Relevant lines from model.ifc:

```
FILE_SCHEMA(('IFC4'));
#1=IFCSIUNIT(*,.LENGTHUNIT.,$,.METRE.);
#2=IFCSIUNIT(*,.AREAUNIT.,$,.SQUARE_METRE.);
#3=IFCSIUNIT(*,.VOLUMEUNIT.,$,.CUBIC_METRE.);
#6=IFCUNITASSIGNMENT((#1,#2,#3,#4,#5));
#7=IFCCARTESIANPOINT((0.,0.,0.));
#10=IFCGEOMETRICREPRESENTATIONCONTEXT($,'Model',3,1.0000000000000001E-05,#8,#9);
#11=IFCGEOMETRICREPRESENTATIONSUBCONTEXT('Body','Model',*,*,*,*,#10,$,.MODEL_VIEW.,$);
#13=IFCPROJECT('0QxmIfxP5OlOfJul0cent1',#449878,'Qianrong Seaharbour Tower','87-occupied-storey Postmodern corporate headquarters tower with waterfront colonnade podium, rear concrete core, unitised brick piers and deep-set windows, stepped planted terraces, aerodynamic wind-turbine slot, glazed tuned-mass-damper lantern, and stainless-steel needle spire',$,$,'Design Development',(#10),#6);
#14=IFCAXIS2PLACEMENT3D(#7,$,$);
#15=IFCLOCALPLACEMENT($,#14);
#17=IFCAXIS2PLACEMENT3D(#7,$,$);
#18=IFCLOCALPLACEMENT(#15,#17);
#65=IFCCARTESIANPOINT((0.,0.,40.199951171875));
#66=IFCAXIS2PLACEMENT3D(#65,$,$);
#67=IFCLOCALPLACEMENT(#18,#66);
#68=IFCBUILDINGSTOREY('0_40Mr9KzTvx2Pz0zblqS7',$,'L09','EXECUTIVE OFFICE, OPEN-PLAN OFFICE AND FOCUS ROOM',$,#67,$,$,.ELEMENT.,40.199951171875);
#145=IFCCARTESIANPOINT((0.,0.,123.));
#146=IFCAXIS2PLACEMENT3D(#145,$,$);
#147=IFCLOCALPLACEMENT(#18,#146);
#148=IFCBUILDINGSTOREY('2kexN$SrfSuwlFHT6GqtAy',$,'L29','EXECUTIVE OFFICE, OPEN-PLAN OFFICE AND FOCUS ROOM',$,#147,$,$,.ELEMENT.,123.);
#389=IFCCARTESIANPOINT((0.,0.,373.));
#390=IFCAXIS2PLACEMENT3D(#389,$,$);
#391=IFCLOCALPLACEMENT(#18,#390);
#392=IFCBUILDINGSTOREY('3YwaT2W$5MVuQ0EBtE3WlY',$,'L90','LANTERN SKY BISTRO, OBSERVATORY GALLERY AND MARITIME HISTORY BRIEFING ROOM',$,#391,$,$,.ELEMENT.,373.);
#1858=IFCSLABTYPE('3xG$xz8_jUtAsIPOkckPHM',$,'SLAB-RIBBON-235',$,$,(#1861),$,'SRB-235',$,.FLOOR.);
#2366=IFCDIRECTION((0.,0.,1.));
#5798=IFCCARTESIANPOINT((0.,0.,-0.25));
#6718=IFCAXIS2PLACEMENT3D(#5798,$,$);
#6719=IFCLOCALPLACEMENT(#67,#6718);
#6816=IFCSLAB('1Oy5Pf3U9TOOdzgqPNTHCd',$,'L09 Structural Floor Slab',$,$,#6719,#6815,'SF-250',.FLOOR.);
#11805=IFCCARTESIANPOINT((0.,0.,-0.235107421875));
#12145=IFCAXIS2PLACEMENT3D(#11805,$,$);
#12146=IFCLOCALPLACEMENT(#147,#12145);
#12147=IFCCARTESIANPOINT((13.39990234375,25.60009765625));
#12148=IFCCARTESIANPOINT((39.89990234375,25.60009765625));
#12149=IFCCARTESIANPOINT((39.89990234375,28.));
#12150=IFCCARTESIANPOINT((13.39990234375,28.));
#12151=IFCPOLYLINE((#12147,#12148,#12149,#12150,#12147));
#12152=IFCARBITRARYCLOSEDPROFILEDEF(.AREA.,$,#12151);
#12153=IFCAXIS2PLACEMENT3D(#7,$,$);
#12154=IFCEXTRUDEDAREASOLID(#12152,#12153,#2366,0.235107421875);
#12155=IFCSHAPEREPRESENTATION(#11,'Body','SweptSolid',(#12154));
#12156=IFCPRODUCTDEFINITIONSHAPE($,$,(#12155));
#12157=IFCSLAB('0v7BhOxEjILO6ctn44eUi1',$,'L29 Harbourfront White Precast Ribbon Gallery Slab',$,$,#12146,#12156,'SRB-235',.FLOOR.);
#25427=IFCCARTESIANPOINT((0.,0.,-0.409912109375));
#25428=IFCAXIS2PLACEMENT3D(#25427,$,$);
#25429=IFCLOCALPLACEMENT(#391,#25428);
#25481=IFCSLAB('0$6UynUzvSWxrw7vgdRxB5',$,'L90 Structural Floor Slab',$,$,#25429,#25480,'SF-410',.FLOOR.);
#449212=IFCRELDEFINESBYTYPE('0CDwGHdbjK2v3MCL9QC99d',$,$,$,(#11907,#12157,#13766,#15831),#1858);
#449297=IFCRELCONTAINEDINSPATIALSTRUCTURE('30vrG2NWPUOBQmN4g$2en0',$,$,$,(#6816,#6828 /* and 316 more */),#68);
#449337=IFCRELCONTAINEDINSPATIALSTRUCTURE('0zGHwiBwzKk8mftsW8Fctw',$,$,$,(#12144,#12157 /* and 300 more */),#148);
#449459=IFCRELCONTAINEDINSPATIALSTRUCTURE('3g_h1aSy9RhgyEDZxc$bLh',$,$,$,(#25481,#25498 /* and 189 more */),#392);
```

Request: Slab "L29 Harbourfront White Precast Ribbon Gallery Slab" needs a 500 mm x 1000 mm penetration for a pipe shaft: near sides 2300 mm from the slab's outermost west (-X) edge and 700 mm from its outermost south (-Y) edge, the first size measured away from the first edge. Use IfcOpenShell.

```python
import numpy as np
import ifcopenshell
import ifcopenshell.api.feature
import ifcopenshell.api.geometry
import ifcopenshell.api.root
import ifcopenshell.geom
import ifcopenshell.util.placement
import ifcopenshell.util.representation
import ifcopenshell.util.shape
import ifcopenshell.util.unit

model = ifcopenshell.open("model.ifc")
unit_scale = ifcopenshell.util.unit.calculate_unit_scale(model)
settings = ifcopenshell.geom.settings()


def volume(element):
    """Net volume in cubic metres, openings subtracted."""
    shape = ifcopenshell.geom.create_shape(settings, element)
    return ifcopenshell.util.shape.get_volume(shape.geometry)


slab = model.by_id(12157)
before = volume(slab)

# Extent in the slab's own axes, in metres. The edges named are its -X and -Y sides.
slab_shape = ifcopenshell.geom.create_shape(settings, slab)
vertices = ifcopenshell.util.shape.get_vertices(slab_shape.geometry)
x_min, y_min, bottom = vertices.min(axis=0)
top = vertices[:, 2].max()

opening = ifcopenshell.api.root.create_entity(model, ifc_class="IfcOpeningElement", name="Pipe shaft opening", predefined_type="OPENING")
context = ifcopenshell.util.representation.get_context(model, "Model", "Body", "MODEL_VIEW")
width, depth = 0.5, 1
outline = [(0.0, 0.0), (width, 0.0), (width, depth), (0.0, depth), (0.0, 0.0)]
# Overshoot both faces by 50 mm so the cut is clean.
shape = ifcopenshell.api.geometry.add_slab_representation(
    model, context=context, depth=top - bottom + 0.1, polyline=outline
)
ifcopenshell.api.geometry.assign_representation(model, product=opening, representation=shape)

matrix = ifcopenshell.util.placement.get_local_placement(slab.ObjectPlacement)
matrix[:, 3] = matrix @ np.append(np.array([x_min + 2.3, y_min + 0.7, bottom - 0.05]) / unit_scale, 1.0)
ifcopenshell.api.geometry.edit_object_placement(model, product=opening, matrix=matrix, is_si=False)
ifcopenshell.api.feature.add_feature(model, feature=opening, element=slab)

after = volume(slab)

print(f"slab volume {before:.3f} -> {after:.3f} m3")

model.write("model_rev.ifc")
```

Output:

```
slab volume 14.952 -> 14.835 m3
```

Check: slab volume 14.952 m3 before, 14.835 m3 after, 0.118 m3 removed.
